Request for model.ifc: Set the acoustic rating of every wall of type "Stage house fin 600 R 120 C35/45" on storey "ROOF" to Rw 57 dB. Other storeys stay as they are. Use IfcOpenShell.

First a look at what the model holds.

```python
import ifcopenshell
import ifcopenshell.util.element

model = ifcopenshell.open("model.ifc")
print(model.schema)
storey = next(s for s in model.by_type("IfcBuildingStorey") if s.Name == "ROOF")
walls = [e for e in ifcopenshell.util.element.get_decomposition(storey) if e.is_a("IfcWall")]
seen = {}
for e in walls:
    element_type = ifcopenshell.util.element.get_type(e)
    key = (element_type.Name if element_type != e and element_type else None, ifcopenshell.util.element.get_pset(e, "Pset_WallCommon", "AcousticRating"))
    seen[key] = seen.get(key, 0) + 1
for (name, value), count in sorted(seen.items(), key=str):
    print(count, "x", name, "|", value)
```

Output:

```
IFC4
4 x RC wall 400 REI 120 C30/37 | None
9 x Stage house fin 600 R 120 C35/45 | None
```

```python
import ifcopenshell
import ifcopenshell.api.pset
import ifcopenshell.util.element

model = ifcopenshell.open("model.ifc")

storey = next(s for s in model.by_type("IfcBuildingStorey") if s.Name == "ROOF")
walls = [e for e in ifcopenshell.util.element.get_decomposition(storey) if e.is_a("IfcWall")]

count = 0
for e in walls:
    element_type = ifcopenshell.util.element.get_type(e)
    if element_type in (None, e) or element_type.Name != "Stage house fin 600 R 120 C35/45":
        continue
    # add_pset returns the element's existing set when there is one.
    pset = ifcopenshell.api.pset.add_pset(model, product=e, name="Pset_WallCommon")
    ifcopenshell.api.pset.edit_pset(model, pset=pset, properties={"AcousticRating": "Rw 57 dB"})
    count += 1

print(count, "walls updated")

model.write("model-out.ifc")
```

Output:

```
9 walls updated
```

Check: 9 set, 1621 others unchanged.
